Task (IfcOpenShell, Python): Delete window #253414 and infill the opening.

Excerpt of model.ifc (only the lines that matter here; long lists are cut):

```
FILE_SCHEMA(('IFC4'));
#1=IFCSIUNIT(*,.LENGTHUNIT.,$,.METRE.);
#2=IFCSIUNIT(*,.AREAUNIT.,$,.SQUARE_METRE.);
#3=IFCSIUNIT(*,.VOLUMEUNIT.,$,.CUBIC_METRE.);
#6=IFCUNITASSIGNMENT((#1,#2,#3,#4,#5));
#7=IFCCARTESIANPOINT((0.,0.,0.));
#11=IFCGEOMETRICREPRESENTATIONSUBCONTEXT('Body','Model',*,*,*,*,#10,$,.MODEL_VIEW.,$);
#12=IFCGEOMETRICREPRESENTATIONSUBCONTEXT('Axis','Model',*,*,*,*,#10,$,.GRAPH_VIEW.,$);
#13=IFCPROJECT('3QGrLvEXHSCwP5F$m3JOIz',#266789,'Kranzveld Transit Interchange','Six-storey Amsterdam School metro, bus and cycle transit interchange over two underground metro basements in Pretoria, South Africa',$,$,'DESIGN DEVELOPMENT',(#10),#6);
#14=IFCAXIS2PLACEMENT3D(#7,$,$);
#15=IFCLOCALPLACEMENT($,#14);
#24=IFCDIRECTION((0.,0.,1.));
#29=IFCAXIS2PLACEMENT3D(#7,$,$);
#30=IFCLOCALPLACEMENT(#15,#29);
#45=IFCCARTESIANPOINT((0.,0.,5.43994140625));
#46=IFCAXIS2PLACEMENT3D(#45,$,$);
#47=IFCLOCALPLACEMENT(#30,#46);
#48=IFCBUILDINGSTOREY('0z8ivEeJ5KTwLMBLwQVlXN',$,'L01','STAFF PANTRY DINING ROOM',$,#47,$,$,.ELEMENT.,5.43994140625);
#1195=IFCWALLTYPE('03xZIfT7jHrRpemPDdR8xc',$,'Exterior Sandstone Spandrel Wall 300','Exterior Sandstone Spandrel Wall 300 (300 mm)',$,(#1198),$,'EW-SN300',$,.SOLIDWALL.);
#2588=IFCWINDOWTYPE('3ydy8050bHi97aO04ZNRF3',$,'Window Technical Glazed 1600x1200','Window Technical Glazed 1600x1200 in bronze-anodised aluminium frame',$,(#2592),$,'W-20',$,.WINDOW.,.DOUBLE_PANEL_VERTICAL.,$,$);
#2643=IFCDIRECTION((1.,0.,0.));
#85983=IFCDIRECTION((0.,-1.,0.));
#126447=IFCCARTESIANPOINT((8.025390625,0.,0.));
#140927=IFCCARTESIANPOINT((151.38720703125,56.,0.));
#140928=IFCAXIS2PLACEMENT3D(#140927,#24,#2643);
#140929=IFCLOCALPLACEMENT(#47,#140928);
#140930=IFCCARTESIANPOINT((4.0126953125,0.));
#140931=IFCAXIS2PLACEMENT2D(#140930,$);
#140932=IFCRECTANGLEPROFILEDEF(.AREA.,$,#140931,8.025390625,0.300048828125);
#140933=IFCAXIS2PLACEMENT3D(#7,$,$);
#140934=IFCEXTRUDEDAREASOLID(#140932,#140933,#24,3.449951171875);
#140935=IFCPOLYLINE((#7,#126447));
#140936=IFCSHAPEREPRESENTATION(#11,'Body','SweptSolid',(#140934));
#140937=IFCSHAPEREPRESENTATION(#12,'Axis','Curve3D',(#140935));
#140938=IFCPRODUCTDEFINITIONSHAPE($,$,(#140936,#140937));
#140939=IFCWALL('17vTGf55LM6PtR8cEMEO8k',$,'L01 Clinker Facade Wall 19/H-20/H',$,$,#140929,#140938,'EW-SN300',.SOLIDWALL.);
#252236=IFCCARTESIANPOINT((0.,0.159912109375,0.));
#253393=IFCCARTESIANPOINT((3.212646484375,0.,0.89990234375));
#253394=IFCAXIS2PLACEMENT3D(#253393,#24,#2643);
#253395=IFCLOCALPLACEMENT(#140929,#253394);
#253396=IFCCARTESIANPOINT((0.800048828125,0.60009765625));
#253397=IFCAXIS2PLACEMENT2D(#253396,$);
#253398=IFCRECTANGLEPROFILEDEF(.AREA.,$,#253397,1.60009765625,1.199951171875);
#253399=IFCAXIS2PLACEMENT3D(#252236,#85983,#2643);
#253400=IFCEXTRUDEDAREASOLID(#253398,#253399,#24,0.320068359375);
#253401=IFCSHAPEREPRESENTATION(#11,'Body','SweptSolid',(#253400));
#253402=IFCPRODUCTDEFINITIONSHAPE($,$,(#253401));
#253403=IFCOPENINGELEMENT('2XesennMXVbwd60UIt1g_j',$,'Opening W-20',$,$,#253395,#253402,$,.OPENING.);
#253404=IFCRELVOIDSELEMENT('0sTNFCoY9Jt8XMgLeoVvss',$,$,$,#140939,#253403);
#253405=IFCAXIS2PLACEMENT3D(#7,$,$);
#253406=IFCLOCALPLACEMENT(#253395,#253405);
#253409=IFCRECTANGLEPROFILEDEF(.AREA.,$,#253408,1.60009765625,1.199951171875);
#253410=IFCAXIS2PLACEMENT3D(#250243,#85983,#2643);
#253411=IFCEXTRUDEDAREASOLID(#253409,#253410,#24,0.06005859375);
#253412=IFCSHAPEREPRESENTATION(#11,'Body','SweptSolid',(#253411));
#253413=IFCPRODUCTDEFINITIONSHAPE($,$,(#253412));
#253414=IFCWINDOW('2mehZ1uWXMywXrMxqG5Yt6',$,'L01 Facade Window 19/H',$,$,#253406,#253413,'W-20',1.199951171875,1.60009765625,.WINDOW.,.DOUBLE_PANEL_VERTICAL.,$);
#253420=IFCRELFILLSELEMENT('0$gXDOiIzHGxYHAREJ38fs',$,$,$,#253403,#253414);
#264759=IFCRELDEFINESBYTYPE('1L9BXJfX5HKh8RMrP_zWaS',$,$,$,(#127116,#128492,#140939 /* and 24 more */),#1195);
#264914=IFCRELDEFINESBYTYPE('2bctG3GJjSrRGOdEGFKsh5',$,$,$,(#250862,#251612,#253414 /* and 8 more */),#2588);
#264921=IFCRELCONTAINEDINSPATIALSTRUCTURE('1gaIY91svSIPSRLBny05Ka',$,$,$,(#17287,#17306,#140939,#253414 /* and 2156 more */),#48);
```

```python
import ifcopenshell
import ifcopenshell.api.feature
import ifcopenshell.api.root
import ifcopenshell.geom
import ifcopenshell.util.shape

model = ifcopenshell.open("model.ifc")
settings = ifcopenshell.geom.settings()


def volume(element):
    """Net volume in cubic metres, openings subtracted."""
    shape = ifcopenshell.geom.create_shape(settings, element)
    return ifcopenshell.util.shape.get_volume(shape.geometry)


window = model.by_guid("2mehZ1uWXMywXrMxqG5Yt6")
opening = window.FillsVoids[0].RelatingOpeningElement
wall = opening.VoidsElements[0].RelatingBuildingElement
before = volume(wall)

ifcopenshell.api.root.remove_product(model, product=window)
ifcopenshell.api.feature.remove_feature(model, feature=opening)

after = volume(wall)

print(f"wall volume {before:.3f} -> {after:.3f} m3")

model.write("model_rev.ifc")
```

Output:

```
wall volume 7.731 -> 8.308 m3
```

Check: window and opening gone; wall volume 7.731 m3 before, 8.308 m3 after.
